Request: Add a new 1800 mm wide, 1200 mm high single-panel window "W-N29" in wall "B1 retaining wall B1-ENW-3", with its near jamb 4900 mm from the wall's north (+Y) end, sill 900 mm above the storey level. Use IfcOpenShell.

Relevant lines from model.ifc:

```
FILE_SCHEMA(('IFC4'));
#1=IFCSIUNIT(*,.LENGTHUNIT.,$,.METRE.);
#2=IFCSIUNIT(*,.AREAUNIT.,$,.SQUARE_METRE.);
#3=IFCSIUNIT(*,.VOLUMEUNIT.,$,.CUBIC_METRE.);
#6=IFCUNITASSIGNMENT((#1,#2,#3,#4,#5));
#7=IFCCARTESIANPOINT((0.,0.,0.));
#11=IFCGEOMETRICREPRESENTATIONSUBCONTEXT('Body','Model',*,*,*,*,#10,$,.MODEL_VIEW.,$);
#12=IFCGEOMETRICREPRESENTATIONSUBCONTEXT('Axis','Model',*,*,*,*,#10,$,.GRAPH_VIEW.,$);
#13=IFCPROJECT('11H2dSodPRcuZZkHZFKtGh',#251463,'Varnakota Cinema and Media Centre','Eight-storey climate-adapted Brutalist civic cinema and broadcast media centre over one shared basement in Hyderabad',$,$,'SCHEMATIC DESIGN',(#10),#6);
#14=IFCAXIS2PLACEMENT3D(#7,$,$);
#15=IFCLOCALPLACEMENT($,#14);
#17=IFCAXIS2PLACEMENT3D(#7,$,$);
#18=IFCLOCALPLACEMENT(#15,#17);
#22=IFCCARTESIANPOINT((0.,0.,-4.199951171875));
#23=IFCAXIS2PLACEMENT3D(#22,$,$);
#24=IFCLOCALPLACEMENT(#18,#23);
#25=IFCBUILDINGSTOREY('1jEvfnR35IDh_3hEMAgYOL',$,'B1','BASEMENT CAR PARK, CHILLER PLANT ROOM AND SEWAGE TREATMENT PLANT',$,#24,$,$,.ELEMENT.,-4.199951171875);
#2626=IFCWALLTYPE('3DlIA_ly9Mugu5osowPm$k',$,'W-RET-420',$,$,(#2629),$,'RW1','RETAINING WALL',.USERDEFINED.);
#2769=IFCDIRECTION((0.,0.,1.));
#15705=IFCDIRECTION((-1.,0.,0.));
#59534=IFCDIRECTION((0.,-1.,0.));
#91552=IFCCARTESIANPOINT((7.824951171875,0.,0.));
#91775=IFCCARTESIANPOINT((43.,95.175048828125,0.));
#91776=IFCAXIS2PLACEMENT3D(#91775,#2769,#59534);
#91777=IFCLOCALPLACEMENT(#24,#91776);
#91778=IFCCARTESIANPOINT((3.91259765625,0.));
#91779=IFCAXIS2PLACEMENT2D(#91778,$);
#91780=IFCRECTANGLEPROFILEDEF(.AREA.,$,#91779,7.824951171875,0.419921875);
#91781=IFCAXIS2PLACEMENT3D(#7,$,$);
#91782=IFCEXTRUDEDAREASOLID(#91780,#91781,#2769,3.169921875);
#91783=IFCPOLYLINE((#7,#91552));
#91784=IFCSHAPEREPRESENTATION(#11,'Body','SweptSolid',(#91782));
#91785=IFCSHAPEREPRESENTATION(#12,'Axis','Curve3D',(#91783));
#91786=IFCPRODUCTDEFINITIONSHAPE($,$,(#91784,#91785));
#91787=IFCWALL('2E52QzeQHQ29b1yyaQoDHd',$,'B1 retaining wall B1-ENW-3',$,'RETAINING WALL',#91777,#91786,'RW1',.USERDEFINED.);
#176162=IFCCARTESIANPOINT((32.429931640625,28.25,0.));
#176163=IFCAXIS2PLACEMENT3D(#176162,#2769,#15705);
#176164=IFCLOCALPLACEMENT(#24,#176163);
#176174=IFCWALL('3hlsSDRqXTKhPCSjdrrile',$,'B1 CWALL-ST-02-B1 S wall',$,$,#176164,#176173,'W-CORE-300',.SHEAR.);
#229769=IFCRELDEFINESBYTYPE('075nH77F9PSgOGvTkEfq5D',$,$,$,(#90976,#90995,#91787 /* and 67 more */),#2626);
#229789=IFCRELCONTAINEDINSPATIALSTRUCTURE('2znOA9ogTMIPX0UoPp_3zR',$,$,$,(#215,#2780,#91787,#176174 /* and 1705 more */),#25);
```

```python
import numpy as np
import ifcopenshell
import ifcopenshell.api.feature
import ifcopenshell.api.geometry
import ifcopenshell.api.root
import ifcopenshell.api.spatial
import ifcopenshell.geom
import ifcopenshell.util.element
import ifcopenshell.util.placement
import ifcopenshell.util.representation
import ifcopenshell.util.shape
import ifcopenshell.util.unit

model = ifcopenshell.open("model.ifc")
unit_scale = ifcopenshell.util.unit.calculate_unit_scale(model)
settings = ifcopenshell.geom.settings()


def volume(element):
    """Net volume in cubic metres, openings subtracted."""
    shape = ifcopenshell.geom.create_shape(settings, element)
    return ifcopenshell.util.shape.get_volume(shape.geometry)


wall = model.by_id(91787)
storey = ifcopenshell.util.element.get_container(wall, ifc_class="IfcBuildingStorey")
context = ifcopenshell.util.representation.get_context(model, "Model", "Body", "MODEL_VIEW")
before = volume(wall)

width, height, from_end, sill = 1.8, 1.2, 4.9, 0.9  # metres

# The wall runs along its own X axis, and the end named is its -X end.
wall_shape = ifcopenshell.geom.create_shape(settings, wall)
x, y, z = ifcopenshell.util.shape.get_vertices(wall_shape.geometry).T
start = x.min() + from_end
face, thickness = float(y.min()), float(y.max() - y.min())
wall_matrix = ifcopenshell.util.placement.get_local_placement(wall.ObjectPlacement)
level = ifcopenshell.util.placement.get_local_placement(storey.ObjectPlacement)[2, 3]


def in_wall(x, y):
    """Placement at x, y metres in the wall's axes, at sill height."""
    matrix = wall_matrix.copy()
    matrix[:, 3] = wall_matrix @ np.array([x / unit_scale, y / unit_scale, 0.0, 1.0])
    matrix[2, 3] = level + sill / unit_scale
    return matrix


# Opening: a box that overshoots both wall faces by 50 mm.
opening = ifcopenshell.api.root.create_entity(model, ifc_class="IfcOpeningElement", predefined_type="OPENING")
box = ifcopenshell.api.geometry.add_wall_representation(
    model, context=context, length=width, height=height, thickness=thickness + 0.1
)
ifcopenshell.api.geometry.assign_representation(model, product=opening, representation=box)
ifcopenshell.api.geometry.edit_object_placement(model, product=opening, matrix=in_wall(start, face - 0.05), is_si=False)
ifcopenshell.api.feature.add_feature(model, feature=opening, element=wall)

window = ifcopenshell.api.root.create_entity(model, ifc_class="IfcWindow", name="W-N29", predefined_type="WINDOW")
window.OverallWidth, window.OverallHeight = width / unit_scale, height / unit_scale
window.PartitioningType = "SINGLE_PANEL"
body = ifcopenshell.api.geometry.add_window_representation(
    model,
    context=context,
    overall_width=window.OverallWidth,
    overall_height=window.OverallHeight,
    partition_type="SINGLE_PANEL",
)
ifcopenshell.api.geometry.assign_representation(model, product=window, representation=body)
ifcopenshell.api.spatial.assign_container(model, products=[window], relating_structure=storey)
ifcopenshell.api.feature.add_filling(model, opening=opening, element=window)

# Centre the window in the wall's thickness.
ifcopenshell.api.geometry.edit_object_placement(model, product=window, matrix=in_wall(start, face), is_si=False)
window_shape = ifcopenshell.geom.create_shape(settings, window)
depth = ifcopenshell.util.shape.get_vertices(window_shape.geometry)[:, 1]
offset = face + thickness / 2 - (depth.min() + depth.max()) / 2
ifcopenshell.api.geometry.edit_object_placement(model, product=window, matrix=in_wall(start, offset), is_si=False)

after = volume(wall)

print(f"wall volume {before:.3f} -> {after:.3f} m3")

model.write("model_rev.ifc")
```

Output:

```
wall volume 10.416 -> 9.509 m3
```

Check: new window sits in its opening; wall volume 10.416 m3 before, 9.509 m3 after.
